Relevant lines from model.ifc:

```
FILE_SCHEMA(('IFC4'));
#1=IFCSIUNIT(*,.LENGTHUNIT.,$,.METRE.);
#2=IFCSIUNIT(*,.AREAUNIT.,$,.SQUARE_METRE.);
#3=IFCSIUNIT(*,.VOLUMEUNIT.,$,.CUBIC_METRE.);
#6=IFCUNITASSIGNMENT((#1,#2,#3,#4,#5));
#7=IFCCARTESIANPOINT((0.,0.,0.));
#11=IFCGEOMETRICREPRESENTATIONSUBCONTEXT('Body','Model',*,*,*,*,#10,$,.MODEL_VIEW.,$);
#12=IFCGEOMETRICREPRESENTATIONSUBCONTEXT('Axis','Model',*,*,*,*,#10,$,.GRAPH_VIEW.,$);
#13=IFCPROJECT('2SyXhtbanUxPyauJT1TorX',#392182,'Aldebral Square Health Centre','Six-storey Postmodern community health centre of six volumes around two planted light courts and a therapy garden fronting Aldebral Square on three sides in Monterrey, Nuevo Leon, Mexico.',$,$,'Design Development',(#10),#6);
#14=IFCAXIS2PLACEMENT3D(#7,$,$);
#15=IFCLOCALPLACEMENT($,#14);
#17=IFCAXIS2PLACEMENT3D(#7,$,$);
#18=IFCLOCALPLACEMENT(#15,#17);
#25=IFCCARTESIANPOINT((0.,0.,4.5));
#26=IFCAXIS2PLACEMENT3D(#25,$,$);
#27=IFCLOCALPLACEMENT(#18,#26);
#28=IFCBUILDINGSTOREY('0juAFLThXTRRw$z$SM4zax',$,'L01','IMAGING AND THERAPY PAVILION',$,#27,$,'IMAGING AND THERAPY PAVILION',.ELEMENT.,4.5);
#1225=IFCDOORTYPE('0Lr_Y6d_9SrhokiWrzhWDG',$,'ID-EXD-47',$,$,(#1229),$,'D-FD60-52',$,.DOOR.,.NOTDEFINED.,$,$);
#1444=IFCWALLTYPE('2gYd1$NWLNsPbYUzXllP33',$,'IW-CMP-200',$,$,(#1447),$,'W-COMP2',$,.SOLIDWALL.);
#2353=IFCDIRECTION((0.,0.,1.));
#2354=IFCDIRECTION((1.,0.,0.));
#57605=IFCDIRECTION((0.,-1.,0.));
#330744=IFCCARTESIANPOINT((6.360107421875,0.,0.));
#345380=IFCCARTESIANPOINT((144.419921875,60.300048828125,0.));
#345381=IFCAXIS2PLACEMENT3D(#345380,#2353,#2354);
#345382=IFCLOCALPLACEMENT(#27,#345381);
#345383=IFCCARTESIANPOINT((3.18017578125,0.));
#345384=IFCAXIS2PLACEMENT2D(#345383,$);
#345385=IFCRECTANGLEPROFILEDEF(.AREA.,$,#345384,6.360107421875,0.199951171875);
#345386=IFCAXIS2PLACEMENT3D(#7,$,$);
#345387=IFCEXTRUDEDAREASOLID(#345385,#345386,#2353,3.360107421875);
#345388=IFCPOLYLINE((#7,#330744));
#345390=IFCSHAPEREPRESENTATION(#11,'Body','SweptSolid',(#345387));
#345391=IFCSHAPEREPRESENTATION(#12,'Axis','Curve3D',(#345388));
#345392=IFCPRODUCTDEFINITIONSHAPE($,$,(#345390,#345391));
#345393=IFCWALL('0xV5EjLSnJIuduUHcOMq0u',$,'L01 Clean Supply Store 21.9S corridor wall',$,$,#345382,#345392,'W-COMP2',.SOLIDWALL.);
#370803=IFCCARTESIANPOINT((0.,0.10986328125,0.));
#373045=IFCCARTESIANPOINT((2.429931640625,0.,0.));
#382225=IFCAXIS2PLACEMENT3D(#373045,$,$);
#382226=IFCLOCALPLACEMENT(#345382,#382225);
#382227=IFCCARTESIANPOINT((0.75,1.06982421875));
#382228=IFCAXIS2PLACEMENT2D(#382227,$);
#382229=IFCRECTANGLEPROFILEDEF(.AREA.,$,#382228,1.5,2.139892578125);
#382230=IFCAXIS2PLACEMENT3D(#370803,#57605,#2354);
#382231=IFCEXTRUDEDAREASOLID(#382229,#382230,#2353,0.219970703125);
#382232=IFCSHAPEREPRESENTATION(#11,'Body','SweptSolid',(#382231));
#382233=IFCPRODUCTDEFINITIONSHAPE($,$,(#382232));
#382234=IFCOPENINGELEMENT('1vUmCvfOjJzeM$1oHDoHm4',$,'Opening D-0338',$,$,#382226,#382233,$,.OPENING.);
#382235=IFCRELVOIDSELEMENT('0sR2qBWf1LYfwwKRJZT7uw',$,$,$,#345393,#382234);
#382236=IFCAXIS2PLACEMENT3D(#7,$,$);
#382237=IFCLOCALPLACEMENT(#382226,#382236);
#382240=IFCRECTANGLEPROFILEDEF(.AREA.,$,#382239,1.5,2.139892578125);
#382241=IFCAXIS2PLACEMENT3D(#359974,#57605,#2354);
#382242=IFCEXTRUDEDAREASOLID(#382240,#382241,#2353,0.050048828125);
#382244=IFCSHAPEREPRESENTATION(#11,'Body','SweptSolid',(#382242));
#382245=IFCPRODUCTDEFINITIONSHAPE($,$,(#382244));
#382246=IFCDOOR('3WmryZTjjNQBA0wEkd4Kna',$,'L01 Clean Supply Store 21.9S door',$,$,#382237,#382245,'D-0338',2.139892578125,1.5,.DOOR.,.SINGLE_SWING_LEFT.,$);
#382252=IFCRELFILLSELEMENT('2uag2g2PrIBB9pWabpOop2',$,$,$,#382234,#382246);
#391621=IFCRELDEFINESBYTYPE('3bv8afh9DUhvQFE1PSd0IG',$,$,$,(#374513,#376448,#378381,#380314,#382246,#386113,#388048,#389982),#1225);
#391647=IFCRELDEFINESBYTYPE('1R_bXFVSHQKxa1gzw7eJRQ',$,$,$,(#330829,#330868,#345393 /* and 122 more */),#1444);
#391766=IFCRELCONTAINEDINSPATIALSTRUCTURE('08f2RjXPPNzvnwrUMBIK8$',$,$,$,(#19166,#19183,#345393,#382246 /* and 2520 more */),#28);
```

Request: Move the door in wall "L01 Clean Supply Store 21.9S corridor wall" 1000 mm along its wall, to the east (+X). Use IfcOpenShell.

```python
import ifcopenshell
import ifcopenshell.api.geometry
import ifcopenshell.util.placement
import ifcopenshell.util.unit

model = ifcopenshell.open("model.ifc")
unit_scale = ifcopenshell.util.unit.calculate_unit_scale(model)

door = model.by_guid("3WmryZTjjNQBA0wEkd4Kna")
opening = door.FillsVoids[0].RelatingOpeningElement
wall = opening.VoidsElements[0].RelatingBuildingElement

wall_matrix = ifcopenshell.util.placement.get_local_placement(wall.ObjectPlacement)
shift = wall_matrix[:3, 0] * 1 / unit_scale
before = ifcopenshell.util.placement.get_local_placement(door.ObjectPlacement)[:3, 3].copy()

# The door is placed relative to its opening, so it follows when the opening moves.
matrix = ifcopenshell.util.placement.get_local_placement(opening.ObjectPlacement)
matrix[:3, 3] += shift
ifcopenshell.api.geometry.edit_object_placement(
    model, product=opening, matrix=matrix, is_si=False, should_transform_children=True
)

after = ifcopenshell.util.placement.get_local_placement(door.ObjectPlacement)[:3, 3]
print("door moved by", (after - before).round(3) + 0.0)

model.write("model_edited.ifc")
```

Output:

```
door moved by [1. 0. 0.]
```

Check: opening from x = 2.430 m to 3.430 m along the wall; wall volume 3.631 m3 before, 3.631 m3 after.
